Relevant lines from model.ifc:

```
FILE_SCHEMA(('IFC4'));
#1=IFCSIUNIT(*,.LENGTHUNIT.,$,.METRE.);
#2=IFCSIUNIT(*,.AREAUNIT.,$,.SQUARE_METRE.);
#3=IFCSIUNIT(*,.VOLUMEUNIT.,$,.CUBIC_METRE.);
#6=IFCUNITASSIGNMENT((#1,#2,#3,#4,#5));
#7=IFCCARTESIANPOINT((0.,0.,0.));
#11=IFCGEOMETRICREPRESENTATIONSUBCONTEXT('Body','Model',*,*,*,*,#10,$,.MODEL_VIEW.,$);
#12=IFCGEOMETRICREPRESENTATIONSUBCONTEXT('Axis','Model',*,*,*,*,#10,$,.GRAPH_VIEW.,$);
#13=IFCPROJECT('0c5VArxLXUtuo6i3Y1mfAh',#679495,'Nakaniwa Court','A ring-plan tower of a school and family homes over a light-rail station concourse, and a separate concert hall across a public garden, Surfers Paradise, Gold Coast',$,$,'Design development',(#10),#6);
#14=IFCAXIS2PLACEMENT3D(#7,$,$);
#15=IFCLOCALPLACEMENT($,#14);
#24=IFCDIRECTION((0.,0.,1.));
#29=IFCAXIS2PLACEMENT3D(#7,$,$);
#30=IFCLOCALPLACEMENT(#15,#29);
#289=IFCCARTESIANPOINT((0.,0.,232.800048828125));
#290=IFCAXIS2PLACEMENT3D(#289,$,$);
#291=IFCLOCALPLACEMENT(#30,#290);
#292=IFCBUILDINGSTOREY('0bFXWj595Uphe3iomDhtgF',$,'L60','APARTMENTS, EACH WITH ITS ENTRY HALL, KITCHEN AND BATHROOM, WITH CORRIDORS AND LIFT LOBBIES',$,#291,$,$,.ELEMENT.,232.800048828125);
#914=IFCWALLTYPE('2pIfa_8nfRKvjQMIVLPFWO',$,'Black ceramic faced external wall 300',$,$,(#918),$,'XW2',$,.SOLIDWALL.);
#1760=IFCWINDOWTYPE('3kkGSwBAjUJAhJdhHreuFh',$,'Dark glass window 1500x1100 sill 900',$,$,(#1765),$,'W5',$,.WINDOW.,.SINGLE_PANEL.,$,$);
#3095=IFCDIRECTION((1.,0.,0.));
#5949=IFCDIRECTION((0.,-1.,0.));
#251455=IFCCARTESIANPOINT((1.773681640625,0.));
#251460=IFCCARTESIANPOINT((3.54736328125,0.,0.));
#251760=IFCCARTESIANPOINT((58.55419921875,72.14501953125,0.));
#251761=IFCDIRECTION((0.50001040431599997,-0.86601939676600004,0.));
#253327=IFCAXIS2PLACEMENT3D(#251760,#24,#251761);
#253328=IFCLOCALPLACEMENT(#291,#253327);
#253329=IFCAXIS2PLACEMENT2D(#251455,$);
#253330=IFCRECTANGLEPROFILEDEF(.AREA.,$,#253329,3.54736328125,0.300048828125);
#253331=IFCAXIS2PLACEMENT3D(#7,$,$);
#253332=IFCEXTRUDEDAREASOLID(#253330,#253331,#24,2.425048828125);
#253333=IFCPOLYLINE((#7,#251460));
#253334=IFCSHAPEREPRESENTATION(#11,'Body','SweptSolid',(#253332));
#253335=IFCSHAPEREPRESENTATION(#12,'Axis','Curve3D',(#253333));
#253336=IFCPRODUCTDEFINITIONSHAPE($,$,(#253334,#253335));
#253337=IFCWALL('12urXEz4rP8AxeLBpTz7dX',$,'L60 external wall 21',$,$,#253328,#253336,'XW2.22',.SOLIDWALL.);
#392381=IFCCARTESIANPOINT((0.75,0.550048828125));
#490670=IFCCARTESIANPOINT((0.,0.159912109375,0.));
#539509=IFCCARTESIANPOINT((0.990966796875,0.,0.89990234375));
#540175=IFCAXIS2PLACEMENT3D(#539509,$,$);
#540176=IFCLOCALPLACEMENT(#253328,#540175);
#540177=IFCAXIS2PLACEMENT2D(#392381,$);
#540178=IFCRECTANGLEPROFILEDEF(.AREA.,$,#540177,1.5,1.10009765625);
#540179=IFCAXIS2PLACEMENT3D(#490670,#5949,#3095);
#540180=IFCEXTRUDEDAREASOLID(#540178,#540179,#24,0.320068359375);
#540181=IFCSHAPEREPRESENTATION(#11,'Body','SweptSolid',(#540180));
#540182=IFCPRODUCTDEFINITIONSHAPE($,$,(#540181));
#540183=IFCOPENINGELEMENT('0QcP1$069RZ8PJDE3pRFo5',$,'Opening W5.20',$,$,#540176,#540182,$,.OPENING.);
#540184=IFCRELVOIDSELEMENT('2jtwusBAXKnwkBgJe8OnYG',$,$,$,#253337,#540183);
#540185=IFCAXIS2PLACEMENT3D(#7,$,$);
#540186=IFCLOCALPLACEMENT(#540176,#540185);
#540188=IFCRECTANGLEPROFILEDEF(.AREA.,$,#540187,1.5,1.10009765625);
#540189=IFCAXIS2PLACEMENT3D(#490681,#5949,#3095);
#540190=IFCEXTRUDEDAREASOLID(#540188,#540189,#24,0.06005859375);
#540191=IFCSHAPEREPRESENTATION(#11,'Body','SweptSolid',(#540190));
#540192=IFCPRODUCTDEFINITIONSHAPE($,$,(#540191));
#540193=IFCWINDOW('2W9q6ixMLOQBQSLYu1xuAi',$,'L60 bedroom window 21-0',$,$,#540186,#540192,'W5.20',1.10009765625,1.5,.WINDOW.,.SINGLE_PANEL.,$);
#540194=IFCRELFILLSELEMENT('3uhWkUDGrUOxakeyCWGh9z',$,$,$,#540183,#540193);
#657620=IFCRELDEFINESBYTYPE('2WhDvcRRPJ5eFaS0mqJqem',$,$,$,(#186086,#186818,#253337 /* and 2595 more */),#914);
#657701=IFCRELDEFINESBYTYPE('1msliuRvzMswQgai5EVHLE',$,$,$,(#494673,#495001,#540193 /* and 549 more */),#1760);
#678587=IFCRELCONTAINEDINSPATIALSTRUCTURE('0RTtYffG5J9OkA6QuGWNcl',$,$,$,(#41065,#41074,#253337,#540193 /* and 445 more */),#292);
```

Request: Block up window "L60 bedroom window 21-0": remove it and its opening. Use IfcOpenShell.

```python
import ifcopenshell
import ifcopenshell.api.feature
import ifcopenshell.api.root
import ifcopenshell.geom
import ifcopenshell.util.shape

model = ifcopenshell.open("model.ifc")
settings = ifcopenshell.geom.settings()


def volume(element):
    """Net volume in cubic metres, openings subtracted."""
    shape = ifcopenshell.geom.create_shape(settings, element)
    return ifcopenshell.util.shape.get_volume(shape.geometry)


window = model.by_guid("2W9q6ixMLOQBQSLYu1xuAi")
opening = window.FillsVoids[0].RelatingOpeningElement
wall = opening.VoidsElements[0].RelatingBuildingElement
before = volume(wall)

ifcopenshell.api.root.remove_product(model, product=window)
ifcopenshell.api.feature.remove_feature(model, feature=opening)

after = volume(wall)

print(f"wall volume {before:.3f} -> {after:.3f} m3")

model.write("model_rev.ifc")
```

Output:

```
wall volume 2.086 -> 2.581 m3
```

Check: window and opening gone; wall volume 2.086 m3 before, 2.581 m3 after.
